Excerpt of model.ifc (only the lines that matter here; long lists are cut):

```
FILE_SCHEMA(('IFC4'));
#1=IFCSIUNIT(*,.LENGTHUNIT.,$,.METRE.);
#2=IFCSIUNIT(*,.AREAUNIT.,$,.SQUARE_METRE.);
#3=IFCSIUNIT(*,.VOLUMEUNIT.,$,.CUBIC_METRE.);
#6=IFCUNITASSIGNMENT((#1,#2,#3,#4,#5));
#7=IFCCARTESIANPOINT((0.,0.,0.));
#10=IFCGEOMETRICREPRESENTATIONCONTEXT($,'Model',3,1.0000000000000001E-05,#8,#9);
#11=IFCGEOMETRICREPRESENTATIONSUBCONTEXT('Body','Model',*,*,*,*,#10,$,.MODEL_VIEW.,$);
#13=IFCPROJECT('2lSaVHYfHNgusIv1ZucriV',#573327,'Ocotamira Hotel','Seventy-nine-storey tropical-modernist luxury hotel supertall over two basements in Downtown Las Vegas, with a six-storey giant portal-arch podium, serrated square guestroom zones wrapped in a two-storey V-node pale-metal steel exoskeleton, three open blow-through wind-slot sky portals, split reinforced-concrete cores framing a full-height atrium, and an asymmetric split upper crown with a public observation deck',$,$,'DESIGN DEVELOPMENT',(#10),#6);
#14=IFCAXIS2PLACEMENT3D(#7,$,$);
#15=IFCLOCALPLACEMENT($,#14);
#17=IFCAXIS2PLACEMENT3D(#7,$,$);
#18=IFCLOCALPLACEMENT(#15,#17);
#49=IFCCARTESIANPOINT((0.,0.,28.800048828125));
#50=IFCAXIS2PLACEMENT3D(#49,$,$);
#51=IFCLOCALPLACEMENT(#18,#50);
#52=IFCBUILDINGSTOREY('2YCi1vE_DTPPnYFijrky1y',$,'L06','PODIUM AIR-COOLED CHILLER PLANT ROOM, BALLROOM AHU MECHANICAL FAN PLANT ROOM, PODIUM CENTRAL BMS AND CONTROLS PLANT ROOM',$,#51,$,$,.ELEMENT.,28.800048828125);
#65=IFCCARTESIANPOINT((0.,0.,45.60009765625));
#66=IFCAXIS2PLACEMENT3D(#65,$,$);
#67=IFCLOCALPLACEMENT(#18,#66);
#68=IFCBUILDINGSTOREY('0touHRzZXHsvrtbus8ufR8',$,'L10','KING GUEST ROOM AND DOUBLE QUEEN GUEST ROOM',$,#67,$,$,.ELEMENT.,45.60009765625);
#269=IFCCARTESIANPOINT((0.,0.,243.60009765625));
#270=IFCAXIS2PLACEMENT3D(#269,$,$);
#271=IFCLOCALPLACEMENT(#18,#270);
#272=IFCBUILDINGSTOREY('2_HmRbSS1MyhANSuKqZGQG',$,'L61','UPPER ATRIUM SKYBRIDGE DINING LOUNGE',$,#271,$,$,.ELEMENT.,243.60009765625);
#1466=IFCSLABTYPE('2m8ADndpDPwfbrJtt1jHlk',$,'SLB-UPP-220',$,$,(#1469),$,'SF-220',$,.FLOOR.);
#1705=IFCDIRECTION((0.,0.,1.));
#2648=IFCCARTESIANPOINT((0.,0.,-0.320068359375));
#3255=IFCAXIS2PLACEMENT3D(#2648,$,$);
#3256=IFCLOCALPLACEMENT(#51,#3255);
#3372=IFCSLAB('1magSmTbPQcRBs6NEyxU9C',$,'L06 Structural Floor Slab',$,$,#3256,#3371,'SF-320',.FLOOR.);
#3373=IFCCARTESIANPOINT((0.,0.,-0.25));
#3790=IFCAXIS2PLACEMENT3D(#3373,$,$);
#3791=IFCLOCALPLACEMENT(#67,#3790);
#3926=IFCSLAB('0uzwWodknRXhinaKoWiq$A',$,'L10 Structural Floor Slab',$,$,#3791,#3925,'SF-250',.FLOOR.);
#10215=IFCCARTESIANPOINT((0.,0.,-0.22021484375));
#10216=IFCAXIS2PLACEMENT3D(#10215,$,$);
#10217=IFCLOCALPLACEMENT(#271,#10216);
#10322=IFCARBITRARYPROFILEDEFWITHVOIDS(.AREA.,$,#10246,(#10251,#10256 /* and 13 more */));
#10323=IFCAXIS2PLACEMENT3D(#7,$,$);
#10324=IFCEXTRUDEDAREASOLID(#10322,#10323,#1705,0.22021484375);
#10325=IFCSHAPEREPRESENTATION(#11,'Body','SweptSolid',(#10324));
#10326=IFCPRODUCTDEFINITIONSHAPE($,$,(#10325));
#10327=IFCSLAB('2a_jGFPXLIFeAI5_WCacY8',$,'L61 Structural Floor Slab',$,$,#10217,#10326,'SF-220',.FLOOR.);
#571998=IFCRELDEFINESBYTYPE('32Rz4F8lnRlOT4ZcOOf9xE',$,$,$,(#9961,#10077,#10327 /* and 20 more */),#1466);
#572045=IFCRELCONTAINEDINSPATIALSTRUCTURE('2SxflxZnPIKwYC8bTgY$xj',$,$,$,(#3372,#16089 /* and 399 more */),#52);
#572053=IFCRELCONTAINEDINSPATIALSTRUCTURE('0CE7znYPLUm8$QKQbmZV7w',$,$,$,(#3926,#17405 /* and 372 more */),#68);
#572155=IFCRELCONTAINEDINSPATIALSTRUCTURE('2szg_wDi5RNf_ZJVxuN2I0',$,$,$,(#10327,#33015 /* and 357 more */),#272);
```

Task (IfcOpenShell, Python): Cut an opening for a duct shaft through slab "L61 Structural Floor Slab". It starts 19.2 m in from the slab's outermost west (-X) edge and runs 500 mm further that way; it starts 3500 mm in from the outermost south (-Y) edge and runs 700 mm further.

```python
import numpy as np
import ifcopenshell
import ifcopenshell.api.feature
import ifcopenshell.api.geometry
import ifcopenshell.api.root
import ifcopenshell.geom
import ifcopenshell.util.placement
import ifcopenshell.util.representation
import ifcopenshell.util.shape
import ifcopenshell.util.unit

model = ifcopenshell.open("model.ifc")
unit_scale = ifcopenshell.util.unit.calculate_unit_scale(model)
settings = ifcopenshell.geom.settings()


def volume(element):
    """Net volume in cubic metres, openings subtracted."""
    shape = ifcopenshell.geom.create_shape(settings, element)
    return ifcopenshell.util.shape.get_volume(shape.geometry)


slab = model.by_id(10327)
before = volume(slab)

# Extent in the slab's own axes, in metres. The edges named are its -X and -Y sides.
slab_shape = ifcopenshell.geom.create_shape(settings, slab)
vertices = ifcopenshell.util.shape.get_vertices(slab_shape.geometry)
x_min, y_min, bottom = vertices.min(axis=0)
top = vertices[:, 2].max()

opening = ifcopenshell.api.root.create_entity(model, ifc_class="IfcOpeningElement", name="Duct shaft opening", predefined_type="OPENING")
context = ifcopenshell.util.representation.get_context(model, "Model", "Body", "MODEL_VIEW")
width, depth = 0.5, 0.7
outline = [(0.0, 0.0), (width, 0.0), (width, depth), (0.0, depth), (0.0, 0.0)]
# Overshoot both faces by 50 mm so the cut is clean.
shape = ifcopenshell.api.geometry.add_slab_representation(
    model, context=context, depth=top - bottom + 0.1, polyline=outline
)
ifcopenshell.api.geometry.assign_representation(model, product=opening, representation=shape)

matrix = ifcopenshell.util.placement.get_local_placement(slab.ObjectPlacement)
matrix[:, 3] = matrix @ np.append(np.array([x_min + 19.2, y_min + 3.5, bottom - 0.05]) / unit_scale, 1.0)
ifcopenshell.api.geometry.edit_object_placement(model, product=opening, matrix=matrix, is_si=False)
ifcopenshell.api.feature.add_feature(model, feature=opening, element=slab)

after = volume(slab)

print(f"slab volume {before:.3f} -> {after:.3f} m3")

model.write("model_rev.ifc")
```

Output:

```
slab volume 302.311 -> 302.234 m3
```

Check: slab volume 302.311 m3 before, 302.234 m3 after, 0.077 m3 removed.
